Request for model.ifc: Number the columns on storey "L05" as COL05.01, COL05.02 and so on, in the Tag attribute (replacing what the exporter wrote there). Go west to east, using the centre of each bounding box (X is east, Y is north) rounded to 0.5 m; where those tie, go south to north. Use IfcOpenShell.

First a look at what the model holds.

```python
import ifcopenshell
import ifcopenshell.util.element
import ifcopenshell.util.placement

model = ifcopenshell.open("model.ifc")
print(model.schema)
storey = next(s for s in model.by_type("IfcBuildingStorey") if s.Name == "L05")
columns = [e for e in ifcopenshell.util.element.get_decomposition(storey) if e.is_a("IfcColumn")]
for e in sorted(columns, key=lambda e: e.id()):
    origin = ifcopenshell.util.placement.get_local_placement(e.ObjectPlacement)[:3, 3]
    print(e.id(), e.Tag, e.Name, origin.round(2) + 0.0, sep=" | ")
```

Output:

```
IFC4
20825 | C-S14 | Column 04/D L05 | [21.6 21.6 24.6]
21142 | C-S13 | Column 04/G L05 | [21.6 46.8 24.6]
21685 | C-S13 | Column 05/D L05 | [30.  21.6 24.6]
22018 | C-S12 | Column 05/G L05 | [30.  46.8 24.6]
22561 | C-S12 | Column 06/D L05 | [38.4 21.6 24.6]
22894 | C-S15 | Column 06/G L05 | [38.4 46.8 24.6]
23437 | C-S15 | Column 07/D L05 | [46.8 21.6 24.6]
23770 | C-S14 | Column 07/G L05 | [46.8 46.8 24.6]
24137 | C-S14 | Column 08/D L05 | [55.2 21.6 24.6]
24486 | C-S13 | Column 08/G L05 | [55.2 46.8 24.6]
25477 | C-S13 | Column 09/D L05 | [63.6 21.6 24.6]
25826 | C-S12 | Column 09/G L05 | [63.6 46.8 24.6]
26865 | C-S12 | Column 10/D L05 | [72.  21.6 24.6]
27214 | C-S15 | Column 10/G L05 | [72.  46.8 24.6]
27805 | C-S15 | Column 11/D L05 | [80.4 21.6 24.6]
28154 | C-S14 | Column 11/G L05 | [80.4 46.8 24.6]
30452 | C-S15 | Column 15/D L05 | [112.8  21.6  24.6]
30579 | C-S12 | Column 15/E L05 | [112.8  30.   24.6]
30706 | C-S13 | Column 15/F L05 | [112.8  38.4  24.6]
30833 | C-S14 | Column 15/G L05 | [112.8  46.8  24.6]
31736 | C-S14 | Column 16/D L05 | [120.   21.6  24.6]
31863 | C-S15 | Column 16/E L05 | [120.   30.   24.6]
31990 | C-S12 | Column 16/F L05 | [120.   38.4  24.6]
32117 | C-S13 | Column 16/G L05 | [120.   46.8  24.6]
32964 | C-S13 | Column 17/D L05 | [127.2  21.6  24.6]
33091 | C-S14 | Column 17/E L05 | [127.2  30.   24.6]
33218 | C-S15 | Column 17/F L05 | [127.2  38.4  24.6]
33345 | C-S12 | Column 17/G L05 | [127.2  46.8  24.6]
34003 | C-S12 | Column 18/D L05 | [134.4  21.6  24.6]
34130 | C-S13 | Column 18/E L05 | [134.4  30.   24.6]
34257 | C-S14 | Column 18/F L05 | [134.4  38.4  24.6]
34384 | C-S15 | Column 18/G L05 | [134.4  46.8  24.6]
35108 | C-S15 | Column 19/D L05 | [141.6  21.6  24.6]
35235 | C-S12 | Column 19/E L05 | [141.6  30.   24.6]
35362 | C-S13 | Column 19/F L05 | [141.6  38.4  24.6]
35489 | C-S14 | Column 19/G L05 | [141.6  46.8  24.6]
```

```python
import ifcopenshell
import ifcopenshell.geom
import ifcopenshell.util.element
import ifcopenshell.util.shape

model = ifcopenshell.open("model.ifc")
settings = ifcopenshell.geom.settings()
settings.set("use-world-coords", True)


def centre(element):
    shape = ifcopenshell.geom.create_shape(settings, element)
    return ifcopenshell.util.shape.get_bbox_centroid(shape.geometry)


storey = next(s for s in model.by_type("IfcBuildingStorey") if s.Name == "L05")
columns = [e for e in ifcopenshell.util.element.get_decomposition(storey) if e.is_a("IfcColumn")]

# Insertion points can sit at a corner or the storey origin, so sort by the geometry (in metres).
centres = {e: centre(e) for e in columns}
columns.sort(key=lambda e: (round(centres[e][0] / 0.5), centres[e][1]))

for i, e in enumerate(columns, start=1):
    number = f"COL05.{i:02d}"
    e.Tag = number
    print(e.id(), number)

model.write("model_edited.ifc")
```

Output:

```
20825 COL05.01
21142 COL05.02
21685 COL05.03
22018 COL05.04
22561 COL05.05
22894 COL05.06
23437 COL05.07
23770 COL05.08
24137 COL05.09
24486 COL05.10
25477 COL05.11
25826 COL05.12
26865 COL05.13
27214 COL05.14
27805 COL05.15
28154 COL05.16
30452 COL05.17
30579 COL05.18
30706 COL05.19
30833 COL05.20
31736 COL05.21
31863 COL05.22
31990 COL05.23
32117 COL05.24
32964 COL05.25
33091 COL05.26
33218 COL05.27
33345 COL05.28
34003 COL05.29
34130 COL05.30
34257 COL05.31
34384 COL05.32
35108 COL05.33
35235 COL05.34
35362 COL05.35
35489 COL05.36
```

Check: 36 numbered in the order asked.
